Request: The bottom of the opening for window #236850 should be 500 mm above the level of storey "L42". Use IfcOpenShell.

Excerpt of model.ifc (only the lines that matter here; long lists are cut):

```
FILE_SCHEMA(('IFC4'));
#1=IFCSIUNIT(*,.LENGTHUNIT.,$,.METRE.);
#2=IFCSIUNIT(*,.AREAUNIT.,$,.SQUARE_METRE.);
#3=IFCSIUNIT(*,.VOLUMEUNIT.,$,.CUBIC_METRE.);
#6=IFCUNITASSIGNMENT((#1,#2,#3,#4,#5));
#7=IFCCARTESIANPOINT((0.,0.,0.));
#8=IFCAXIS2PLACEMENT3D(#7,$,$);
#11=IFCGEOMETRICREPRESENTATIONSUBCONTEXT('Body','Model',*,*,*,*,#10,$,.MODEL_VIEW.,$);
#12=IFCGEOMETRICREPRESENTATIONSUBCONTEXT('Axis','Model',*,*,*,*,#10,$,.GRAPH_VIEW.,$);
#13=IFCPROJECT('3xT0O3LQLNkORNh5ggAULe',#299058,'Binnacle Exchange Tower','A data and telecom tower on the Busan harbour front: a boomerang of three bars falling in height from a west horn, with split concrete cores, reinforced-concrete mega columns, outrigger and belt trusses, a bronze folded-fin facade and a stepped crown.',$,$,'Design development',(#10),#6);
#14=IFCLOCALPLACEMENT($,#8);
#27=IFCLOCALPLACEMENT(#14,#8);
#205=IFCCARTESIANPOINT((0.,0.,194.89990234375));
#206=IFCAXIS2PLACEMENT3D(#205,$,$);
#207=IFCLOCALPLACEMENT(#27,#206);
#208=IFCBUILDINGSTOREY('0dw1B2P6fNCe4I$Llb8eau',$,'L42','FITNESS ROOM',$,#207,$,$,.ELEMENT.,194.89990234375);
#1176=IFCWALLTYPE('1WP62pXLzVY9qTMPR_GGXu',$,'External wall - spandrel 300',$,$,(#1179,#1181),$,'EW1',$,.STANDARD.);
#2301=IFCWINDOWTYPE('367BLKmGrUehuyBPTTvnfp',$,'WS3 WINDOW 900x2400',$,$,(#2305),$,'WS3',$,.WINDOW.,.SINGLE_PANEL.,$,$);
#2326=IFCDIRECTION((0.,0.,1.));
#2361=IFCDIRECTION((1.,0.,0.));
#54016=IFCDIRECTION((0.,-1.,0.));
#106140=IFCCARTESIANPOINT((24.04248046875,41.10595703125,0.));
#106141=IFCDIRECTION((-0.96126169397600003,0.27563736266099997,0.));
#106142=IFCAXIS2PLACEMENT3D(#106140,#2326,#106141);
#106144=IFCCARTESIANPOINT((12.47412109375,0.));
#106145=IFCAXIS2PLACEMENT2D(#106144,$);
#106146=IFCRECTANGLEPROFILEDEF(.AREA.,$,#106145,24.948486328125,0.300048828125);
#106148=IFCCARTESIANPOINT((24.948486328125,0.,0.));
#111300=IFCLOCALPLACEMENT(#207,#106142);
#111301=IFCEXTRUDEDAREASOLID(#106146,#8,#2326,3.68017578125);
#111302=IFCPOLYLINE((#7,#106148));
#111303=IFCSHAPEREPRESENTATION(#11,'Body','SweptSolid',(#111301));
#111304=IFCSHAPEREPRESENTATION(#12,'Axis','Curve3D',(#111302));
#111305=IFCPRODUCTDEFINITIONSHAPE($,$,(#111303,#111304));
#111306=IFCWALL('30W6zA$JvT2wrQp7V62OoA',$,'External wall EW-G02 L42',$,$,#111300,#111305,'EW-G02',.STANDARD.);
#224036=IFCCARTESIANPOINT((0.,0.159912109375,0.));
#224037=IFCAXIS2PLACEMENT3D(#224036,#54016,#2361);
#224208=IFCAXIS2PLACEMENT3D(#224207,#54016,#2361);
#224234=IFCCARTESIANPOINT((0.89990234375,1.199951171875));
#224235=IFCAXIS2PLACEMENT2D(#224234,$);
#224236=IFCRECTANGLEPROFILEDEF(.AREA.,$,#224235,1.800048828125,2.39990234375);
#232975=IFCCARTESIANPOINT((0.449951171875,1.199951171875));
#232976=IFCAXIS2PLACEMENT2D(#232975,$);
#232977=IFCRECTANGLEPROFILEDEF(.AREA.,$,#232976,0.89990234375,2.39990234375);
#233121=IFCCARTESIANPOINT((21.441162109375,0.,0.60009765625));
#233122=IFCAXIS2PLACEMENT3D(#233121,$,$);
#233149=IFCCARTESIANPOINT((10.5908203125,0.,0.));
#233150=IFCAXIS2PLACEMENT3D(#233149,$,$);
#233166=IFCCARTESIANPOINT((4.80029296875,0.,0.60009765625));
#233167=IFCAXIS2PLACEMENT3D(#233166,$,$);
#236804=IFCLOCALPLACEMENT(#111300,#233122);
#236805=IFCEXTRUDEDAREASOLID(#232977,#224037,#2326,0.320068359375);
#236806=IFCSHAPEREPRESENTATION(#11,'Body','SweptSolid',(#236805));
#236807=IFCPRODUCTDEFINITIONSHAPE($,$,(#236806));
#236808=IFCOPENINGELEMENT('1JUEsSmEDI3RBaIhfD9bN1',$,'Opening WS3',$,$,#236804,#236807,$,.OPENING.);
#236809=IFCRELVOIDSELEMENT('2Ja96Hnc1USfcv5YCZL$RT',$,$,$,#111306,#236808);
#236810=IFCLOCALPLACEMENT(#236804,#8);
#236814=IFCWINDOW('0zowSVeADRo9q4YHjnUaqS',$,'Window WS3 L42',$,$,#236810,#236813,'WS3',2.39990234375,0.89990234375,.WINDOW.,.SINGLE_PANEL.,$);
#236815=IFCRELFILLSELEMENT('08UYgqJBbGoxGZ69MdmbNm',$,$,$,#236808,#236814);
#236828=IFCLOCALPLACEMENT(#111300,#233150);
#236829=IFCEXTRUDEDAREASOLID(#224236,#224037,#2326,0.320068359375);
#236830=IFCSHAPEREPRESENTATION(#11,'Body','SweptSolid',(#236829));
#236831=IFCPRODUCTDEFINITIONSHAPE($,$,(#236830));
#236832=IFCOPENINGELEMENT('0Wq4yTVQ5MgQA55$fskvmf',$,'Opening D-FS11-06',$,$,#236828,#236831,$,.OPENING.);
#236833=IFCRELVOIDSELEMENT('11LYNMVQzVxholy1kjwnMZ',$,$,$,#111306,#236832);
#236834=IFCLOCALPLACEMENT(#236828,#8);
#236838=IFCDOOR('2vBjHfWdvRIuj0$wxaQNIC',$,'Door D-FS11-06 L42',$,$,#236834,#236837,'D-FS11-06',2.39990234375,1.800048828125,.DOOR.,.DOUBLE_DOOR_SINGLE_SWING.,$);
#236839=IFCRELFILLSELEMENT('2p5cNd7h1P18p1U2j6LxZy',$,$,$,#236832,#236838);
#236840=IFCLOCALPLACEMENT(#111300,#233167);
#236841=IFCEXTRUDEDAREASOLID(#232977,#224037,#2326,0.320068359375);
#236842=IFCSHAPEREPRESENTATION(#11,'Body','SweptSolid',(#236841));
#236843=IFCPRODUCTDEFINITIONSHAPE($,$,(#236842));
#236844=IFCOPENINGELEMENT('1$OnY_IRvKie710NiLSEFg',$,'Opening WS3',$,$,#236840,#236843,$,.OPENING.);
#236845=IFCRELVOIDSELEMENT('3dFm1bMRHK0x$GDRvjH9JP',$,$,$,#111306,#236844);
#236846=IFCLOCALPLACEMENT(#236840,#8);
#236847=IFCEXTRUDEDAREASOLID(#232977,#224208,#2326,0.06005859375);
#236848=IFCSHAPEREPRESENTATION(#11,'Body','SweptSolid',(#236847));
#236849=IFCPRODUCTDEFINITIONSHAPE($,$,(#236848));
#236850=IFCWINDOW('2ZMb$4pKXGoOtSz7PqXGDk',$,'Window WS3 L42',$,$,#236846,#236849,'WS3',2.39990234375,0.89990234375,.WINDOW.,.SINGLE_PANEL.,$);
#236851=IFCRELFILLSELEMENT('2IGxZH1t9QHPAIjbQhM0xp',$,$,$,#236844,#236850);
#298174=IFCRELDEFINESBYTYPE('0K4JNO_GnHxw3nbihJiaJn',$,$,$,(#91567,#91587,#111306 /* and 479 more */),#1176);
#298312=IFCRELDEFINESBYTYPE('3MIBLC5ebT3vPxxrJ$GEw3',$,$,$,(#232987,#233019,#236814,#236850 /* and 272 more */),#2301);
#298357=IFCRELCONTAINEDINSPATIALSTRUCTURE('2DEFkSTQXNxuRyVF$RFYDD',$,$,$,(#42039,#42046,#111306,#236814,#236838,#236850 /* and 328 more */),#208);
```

```python
import numpy as np
import ifcopenshell
import ifcopenshell.api.geometry
import ifcopenshell.geom
import ifcopenshell.util.element
import ifcopenshell.util.placement
import ifcopenshell.util.shape
import ifcopenshell.util.unit

model = ifcopenshell.open("model.ifc")
unit_scale = ifcopenshell.util.unit.calculate_unit_scale(model)

window = model.by_guid("2ZMb$4pKXGoOtSz7PqXGDk")
opening = window.FillsVoids[0].RelatingOpeningElement
storey = ifcopenshell.util.element.get_container(window, ifc_class="IfcBuildingStorey")
level = ifcopenshell.util.placement.get_local_placement(storey.ObjectPlacement)[2, 3]

# The opening's origin need not be at the sill, so measure its lowest point.
shape = ifcopenshell.geom.create_shape(ifcopenshell.geom.settings(), opening)
bottom = ifcopenshell.util.shape.get_shape_bottom_elevation(shape, shape.geometry) / unit_scale
dz = level + 0.5 - bottom

shift = np.array([0.0, 0.0, dz])
# The window is placed relative to its opening, so it follows when the opening moves.
matrix = ifcopenshell.util.placement.get_local_placement(opening.ObjectPlacement)
matrix[:3, 3] += shift
ifcopenshell.api.geometry.edit_object_placement(
    model, product=opening, matrix=matrix, is_si=False, should_transform_children=True
)

print(f"moved by {dz * unit_scale:+.3f} m")

model.write("model_updated.ifc")
```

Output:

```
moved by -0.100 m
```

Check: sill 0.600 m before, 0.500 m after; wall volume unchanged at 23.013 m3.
